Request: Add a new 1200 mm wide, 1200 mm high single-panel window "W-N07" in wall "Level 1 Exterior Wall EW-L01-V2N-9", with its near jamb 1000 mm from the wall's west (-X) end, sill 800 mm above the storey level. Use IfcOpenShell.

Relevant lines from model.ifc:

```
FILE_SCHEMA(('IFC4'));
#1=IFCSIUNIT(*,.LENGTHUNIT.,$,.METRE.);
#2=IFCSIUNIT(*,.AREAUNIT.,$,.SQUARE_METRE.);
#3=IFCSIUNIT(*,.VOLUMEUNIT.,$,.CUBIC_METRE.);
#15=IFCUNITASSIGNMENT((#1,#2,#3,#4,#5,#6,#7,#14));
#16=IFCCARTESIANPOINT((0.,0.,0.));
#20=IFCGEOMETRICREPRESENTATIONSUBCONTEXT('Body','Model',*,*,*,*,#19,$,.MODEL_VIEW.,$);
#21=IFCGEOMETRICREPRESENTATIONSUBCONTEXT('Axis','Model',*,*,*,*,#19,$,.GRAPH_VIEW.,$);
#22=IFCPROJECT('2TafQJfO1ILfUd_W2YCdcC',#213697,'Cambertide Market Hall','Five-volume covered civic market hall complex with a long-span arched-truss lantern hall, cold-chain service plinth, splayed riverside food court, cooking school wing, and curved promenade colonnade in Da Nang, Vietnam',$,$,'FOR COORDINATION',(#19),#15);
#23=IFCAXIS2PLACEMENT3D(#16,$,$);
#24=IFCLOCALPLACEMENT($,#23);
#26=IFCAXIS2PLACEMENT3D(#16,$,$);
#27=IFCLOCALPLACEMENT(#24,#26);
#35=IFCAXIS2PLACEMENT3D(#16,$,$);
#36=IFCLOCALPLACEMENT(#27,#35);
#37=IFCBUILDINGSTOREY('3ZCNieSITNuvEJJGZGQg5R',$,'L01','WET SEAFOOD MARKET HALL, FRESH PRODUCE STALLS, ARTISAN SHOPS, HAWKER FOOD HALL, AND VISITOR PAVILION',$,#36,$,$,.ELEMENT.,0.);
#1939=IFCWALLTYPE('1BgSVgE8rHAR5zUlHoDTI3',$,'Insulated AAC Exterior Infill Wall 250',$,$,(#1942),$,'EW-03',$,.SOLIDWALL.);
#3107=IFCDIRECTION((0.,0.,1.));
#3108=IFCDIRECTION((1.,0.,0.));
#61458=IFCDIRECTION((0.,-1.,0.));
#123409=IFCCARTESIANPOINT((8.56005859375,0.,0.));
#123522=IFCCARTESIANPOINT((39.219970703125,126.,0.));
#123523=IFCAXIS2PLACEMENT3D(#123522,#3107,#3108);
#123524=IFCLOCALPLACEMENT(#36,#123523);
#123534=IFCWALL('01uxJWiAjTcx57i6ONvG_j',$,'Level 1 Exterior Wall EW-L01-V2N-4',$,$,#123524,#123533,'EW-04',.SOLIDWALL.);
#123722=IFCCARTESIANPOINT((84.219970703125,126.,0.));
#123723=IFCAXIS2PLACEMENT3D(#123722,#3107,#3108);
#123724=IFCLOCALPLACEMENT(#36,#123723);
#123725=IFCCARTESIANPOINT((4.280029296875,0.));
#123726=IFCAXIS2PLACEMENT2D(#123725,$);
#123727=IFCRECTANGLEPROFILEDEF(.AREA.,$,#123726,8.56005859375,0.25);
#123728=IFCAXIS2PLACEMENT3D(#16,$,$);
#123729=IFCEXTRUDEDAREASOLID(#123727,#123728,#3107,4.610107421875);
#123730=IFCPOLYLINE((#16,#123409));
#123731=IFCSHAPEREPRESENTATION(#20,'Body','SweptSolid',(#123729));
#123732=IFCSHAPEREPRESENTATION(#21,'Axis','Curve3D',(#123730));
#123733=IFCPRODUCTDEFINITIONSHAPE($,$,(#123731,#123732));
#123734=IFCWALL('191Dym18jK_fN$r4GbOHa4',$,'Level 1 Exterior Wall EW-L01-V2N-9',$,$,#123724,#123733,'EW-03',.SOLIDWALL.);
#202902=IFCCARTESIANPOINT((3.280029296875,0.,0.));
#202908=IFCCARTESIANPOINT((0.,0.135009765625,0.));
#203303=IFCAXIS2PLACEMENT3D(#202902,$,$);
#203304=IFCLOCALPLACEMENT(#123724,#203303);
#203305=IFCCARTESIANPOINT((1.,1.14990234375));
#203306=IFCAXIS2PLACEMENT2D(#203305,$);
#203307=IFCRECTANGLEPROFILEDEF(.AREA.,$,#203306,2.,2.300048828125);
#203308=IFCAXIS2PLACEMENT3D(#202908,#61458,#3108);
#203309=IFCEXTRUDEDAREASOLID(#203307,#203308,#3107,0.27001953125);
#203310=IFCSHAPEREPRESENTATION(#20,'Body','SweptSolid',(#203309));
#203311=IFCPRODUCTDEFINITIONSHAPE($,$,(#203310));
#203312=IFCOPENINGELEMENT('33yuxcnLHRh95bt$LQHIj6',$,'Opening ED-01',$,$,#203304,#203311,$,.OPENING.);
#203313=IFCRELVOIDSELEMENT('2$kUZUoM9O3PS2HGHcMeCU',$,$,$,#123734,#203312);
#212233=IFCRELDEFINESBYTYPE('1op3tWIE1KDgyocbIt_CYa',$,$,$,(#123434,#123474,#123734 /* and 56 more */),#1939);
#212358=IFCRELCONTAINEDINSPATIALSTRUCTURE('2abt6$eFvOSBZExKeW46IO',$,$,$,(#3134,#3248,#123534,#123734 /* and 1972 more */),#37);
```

```python
import numpy as np
import ifcopenshell
import ifcopenshell.api.feature
import ifcopenshell.api.geometry
import ifcopenshell.api.root
import ifcopenshell.api.spatial
import ifcopenshell.geom
import ifcopenshell.util.element
import ifcopenshell.util.placement
import ifcopenshell.util.representation
import ifcopenshell.util.shape
import ifcopenshell.util.unit

model = ifcopenshell.open("model.ifc")
unit_scale = ifcopenshell.util.unit.calculate_unit_scale(model)
settings = ifcopenshell.geom.settings()


def volume(element):
    """Net volume in cubic metres, openings subtracted."""
    shape = ifcopenshell.geom.create_shape(settings, element)
    return ifcopenshell.util.shape.get_volume(shape.geometry)


wall = model.by_guid("191Dym18jK_fN$r4GbOHa4")
storey = ifcopenshell.util.element.get_container(wall, ifc_class="IfcBuildingStorey")
context = ifcopenshell.util.representation.get_context(model, "Model", "Body", "MODEL_VIEW")
before = volume(wall)

width, height, from_end, sill = 1.2, 1.2, 1, 0.8  # metres

# The wall runs along its own X axis, and the end named is its -X end.
wall_shape = ifcopenshell.geom.create_shape(settings, wall)
x, y, z = ifcopenshell.util.shape.get_vertices(wall_shape.geometry).T
start = x.min() + from_end
face, thickness = float(y.min()), float(y.max() - y.min())
wall_matrix = ifcopenshell.util.placement.get_local_placement(wall.ObjectPlacement)
level = ifcopenshell.util.placement.get_local_placement(storey.ObjectPlacement)[2, 3]


def in_wall(x, y):
    """Placement at x, y metres in the wall's axes, at sill height."""
    matrix = wall_matrix.copy()
    matrix[:, 3] = wall_matrix @ np.array([x / unit_scale, y / unit_scale, 0.0, 1.0])
    matrix[2, 3] = level + sill / unit_scale
    return matrix


# Opening: a box that overshoots both wall faces by 50 mm.
opening = ifcopenshell.api.root.create_entity(model, ifc_class="IfcOpeningElement", predefined_type="OPENING")
box = ifcopenshell.api.geometry.add_wall_representation(
    model, context=context, length=width, height=height, thickness=thickness + 0.1
)
ifcopenshell.api.geometry.assign_representation(model, product=opening, representation=box)
ifcopenshell.api.geometry.edit_object_placement(model, product=opening, matrix=in_wall(start, face - 0.05), is_si=False)
ifcopenshell.api.feature.add_feature(model, feature=opening, element=wall)

window = ifcopenshell.api.root.create_entity(model, ifc_class="IfcWindow", name="W-N07", predefined_type="WINDOW")
window.OverallWidth, window.OverallHeight = width / unit_scale, height / unit_scale
window.PartitioningType = "SINGLE_PANEL"
body = ifcopenshell.api.geometry.add_window_representation(
    model,
    context=context,
    overall_width=window.OverallWidth,
    overall_height=window.OverallHeight,
    partition_type="SINGLE_PANEL",
)
ifcopenshell.api.geometry.assign_representation(model, product=window, representation=body)
ifcopenshell.api.spatial.assign_container(model, products=[window], relating_structure=storey)
ifcopenshell.api.feature.add_filling(model, opening=opening, element=window)

# Centre the window in the wall's thickness.
ifcopenshell.api.geometry.edit_object_placement(model, product=window, matrix=in_wall(start, face), is_si=False)
window_shape = ifcopenshell.geom.create_shape(settings, window)
depth = ifcopenshell.util.shape.get_vertices(window_shape.geometry)[:, 1]
offset = face + thickness / 2 - (depth.min() + depth.max()) / 2
ifcopenshell.api.geometry.edit_object_placement(model, product=window, matrix=in_wall(start, offset), is_si=False)

after = volume(wall)

print(f"wall volume {before:.3f} -> {after:.3f} m3")

model.write("model-out.ifc")
```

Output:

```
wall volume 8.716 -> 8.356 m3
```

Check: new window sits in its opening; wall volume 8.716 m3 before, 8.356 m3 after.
